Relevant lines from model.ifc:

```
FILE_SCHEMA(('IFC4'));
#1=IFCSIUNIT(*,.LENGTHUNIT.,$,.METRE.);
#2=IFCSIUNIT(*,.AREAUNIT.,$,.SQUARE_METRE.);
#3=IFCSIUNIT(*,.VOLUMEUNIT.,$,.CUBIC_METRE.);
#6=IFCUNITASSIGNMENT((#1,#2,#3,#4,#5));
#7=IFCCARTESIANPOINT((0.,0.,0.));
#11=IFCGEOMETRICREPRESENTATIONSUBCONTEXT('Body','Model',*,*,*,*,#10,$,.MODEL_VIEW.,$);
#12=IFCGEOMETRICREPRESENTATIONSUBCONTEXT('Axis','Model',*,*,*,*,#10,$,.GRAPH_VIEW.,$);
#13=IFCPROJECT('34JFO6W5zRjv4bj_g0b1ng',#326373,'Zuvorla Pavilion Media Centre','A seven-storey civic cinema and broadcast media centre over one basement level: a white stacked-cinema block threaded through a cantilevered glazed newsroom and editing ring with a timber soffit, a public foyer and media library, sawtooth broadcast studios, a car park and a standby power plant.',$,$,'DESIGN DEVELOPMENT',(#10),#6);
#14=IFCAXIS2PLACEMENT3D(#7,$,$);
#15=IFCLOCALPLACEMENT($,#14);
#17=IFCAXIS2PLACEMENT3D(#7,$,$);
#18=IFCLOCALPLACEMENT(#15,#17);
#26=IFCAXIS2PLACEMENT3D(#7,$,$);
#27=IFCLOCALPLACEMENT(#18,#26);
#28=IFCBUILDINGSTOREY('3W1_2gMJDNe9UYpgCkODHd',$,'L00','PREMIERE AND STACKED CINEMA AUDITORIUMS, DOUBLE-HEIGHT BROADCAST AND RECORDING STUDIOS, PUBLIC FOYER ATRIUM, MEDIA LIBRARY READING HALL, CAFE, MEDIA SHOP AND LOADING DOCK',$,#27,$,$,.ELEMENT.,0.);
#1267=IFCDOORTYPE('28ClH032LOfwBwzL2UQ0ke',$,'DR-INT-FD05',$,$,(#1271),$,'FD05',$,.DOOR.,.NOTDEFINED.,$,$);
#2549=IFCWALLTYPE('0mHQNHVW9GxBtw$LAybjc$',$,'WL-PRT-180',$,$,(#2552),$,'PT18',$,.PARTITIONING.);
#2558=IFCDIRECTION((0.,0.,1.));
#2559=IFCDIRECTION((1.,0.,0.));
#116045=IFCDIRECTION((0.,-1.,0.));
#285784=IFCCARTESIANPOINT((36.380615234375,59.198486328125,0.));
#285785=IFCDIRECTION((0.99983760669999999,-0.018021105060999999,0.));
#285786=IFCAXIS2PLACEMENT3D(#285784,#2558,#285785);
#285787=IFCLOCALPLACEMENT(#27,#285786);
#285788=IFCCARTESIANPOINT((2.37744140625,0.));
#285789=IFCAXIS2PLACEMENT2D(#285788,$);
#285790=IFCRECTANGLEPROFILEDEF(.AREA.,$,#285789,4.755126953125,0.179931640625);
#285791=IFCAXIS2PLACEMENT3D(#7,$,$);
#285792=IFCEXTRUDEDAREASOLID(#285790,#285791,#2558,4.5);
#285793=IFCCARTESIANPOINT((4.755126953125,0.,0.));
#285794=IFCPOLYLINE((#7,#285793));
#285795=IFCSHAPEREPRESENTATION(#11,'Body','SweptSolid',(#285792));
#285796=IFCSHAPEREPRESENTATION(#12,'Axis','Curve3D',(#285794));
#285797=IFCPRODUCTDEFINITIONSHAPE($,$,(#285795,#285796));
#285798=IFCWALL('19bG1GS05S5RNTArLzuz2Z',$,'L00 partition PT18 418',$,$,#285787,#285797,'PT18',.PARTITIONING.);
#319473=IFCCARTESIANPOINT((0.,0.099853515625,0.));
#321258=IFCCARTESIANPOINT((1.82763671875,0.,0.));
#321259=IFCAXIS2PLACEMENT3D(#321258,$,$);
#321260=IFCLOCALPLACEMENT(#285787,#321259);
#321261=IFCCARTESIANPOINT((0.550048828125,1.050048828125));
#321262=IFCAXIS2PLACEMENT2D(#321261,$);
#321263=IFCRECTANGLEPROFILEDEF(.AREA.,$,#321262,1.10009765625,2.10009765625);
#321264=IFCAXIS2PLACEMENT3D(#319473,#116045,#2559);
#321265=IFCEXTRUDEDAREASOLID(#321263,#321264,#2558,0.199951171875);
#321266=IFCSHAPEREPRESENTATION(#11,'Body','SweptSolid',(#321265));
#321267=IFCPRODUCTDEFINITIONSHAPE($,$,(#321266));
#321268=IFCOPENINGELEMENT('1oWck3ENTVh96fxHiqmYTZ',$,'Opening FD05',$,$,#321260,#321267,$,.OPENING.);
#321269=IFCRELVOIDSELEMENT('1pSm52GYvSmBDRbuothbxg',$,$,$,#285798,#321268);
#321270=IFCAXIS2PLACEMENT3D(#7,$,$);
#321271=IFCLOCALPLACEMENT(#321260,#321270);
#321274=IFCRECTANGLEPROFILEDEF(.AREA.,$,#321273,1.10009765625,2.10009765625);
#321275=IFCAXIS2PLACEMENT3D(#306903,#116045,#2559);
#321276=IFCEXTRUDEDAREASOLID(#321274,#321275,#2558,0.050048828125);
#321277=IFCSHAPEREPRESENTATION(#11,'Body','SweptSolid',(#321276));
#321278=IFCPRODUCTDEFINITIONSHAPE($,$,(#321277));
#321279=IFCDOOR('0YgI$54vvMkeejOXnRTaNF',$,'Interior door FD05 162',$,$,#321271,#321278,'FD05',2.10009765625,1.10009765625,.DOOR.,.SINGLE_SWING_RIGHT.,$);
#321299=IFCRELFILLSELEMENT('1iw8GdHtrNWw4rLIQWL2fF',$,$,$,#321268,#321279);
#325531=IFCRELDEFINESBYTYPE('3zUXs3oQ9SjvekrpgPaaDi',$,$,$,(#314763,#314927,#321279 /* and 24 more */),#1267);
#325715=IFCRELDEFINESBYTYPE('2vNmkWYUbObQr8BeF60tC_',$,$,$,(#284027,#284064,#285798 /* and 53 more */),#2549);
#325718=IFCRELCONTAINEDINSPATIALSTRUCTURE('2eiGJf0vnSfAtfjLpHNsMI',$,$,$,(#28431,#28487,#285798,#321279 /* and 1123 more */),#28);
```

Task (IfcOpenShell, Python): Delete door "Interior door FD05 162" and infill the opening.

```python
import ifcopenshell
import ifcopenshell.api.feature
import ifcopenshell.api.root
import ifcopenshell.geom
import ifcopenshell.util.shape

model = ifcopenshell.open("model.ifc")
settings = ifcopenshell.geom.settings()


def volume(element):
    """Net volume in cubic metres, openings subtracted."""
    shape = ifcopenshell.geom.create_shape(settings, element)
    return ifcopenshell.util.shape.get_volume(shape.geometry)


door = model.by_guid("0YgI$54vvMkeejOXnRTaNF")
opening = door.FillsVoids[0].RelatingOpeningElement
wall = opening.VoidsElements[0].RelatingBuildingElement
before = volume(wall)

ifcopenshell.api.root.remove_product(model, product=door)
ifcopenshell.api.feature.remove_feature(model, feature=opening)

after = volume(wall)

print(f"wall volume {before:.3f} -> {after:.3f} m3")

model.write("model_updated.ifc")
```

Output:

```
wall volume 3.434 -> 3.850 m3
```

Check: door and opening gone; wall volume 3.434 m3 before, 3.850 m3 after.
